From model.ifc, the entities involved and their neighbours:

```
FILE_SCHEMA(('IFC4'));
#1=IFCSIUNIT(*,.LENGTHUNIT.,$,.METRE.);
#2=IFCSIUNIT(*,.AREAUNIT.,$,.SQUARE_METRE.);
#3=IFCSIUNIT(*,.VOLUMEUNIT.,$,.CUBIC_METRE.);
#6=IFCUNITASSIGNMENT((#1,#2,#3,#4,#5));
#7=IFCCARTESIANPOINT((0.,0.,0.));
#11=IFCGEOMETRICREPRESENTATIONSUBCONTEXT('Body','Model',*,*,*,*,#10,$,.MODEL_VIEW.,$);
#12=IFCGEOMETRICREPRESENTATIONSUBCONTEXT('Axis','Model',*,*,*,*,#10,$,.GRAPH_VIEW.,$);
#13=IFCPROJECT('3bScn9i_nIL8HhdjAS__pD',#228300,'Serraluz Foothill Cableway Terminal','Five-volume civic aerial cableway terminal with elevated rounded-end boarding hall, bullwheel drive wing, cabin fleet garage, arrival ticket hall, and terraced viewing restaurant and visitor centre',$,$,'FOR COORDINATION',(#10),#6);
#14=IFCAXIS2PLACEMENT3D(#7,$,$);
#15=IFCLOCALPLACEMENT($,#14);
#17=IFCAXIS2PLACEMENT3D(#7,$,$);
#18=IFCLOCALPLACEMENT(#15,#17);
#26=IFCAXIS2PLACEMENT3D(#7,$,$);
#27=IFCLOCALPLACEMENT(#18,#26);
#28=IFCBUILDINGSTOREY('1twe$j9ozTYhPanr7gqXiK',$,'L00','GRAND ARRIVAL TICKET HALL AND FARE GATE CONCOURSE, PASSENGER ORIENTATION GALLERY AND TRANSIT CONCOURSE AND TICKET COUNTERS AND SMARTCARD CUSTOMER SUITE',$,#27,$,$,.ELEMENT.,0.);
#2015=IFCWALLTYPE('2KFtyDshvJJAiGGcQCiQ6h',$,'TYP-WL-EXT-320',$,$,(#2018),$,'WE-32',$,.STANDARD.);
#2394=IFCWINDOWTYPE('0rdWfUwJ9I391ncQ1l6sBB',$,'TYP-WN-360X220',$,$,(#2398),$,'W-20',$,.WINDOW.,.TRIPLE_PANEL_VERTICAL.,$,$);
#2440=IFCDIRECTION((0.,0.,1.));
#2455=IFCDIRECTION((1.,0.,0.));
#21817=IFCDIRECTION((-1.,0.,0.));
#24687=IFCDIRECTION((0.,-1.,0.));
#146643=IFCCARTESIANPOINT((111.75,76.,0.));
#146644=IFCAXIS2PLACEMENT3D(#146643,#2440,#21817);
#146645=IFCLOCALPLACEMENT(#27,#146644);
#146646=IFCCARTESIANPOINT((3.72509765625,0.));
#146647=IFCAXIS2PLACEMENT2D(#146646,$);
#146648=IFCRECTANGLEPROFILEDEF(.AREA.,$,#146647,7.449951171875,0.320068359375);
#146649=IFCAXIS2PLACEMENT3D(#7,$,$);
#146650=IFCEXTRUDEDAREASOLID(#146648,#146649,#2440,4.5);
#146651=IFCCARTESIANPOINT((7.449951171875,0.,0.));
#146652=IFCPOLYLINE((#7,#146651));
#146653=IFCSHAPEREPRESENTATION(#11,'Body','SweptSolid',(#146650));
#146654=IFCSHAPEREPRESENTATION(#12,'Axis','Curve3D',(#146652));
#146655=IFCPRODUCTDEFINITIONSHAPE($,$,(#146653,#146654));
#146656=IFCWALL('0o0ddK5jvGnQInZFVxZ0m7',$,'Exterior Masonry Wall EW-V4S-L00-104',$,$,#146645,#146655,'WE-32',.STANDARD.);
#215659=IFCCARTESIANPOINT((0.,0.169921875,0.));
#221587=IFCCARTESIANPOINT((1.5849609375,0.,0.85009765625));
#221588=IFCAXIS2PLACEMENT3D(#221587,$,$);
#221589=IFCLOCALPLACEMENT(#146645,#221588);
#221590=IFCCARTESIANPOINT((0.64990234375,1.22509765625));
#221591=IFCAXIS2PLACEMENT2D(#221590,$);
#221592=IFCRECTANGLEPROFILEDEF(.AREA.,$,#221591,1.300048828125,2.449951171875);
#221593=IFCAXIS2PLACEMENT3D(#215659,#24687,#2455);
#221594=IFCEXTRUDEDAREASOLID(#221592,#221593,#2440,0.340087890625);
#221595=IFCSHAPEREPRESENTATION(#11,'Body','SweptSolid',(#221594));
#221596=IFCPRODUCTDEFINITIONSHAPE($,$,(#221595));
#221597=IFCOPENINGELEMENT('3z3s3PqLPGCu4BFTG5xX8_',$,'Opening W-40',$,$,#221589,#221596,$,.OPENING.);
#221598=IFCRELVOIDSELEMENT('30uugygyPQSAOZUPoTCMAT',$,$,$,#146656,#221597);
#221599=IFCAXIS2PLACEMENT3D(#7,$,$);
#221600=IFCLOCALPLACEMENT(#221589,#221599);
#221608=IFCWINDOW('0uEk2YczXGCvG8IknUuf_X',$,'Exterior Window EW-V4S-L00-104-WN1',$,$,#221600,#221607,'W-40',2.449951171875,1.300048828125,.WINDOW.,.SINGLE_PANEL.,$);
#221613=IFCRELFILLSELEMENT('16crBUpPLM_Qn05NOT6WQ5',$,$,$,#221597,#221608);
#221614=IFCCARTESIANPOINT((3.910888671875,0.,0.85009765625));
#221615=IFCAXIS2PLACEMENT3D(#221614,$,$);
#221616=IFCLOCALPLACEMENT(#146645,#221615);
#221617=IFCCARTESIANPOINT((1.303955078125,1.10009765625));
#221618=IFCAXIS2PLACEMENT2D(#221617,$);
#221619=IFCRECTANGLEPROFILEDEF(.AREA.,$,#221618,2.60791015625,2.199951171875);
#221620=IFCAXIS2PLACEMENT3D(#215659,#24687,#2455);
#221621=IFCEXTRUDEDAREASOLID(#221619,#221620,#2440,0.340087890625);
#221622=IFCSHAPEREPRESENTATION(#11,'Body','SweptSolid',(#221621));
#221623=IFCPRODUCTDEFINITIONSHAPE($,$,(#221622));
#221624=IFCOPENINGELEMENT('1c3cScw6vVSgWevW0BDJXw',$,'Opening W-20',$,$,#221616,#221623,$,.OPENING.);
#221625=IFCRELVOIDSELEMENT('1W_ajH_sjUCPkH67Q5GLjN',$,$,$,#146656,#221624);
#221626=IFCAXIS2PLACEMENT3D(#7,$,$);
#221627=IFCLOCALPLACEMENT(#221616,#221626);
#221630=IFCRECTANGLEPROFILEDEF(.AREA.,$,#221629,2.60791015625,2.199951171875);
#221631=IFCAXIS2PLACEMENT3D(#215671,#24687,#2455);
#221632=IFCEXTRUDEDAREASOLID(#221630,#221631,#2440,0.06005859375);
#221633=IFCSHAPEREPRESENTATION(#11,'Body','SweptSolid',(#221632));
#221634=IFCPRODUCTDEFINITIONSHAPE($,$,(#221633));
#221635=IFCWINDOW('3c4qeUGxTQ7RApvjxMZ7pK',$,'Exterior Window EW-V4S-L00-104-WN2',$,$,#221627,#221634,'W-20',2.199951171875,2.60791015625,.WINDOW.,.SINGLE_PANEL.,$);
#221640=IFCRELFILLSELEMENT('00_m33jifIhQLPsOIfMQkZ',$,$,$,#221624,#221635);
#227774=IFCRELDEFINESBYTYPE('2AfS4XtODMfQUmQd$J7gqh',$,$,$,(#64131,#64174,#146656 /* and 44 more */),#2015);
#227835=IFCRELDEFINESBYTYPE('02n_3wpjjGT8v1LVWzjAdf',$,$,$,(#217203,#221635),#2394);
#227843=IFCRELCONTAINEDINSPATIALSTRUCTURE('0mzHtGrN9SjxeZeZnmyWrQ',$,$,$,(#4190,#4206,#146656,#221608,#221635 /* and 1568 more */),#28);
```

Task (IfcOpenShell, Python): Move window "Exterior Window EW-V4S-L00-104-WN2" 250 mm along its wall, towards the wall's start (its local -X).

```python
import ifcopenshell
import ifcopenshell.api.geometry
import ifcopenshell.util.placement
import ifcopenshell.util.unit

model = ifcopenshell.open("model.ifc")
unit_scale = ifcopenshell.util.unit.calculate_unit_scale(model)

window = model.by_guid("3c4qeUGxTQ7RApvjxMZ7pK")
opening = window.FillsVoids[0].RelatingOpeningElement
wall = opening.VoidsElements[0].RelatingBuildingElement

wall_matrix = ifcopenshell.util.placement.get_local_placement(wall.ObjectPlacement)
shift = wall_matrix[:3, 0] * -0.25 / unit_scale
before = ifcopenshell.util.placement.get_local_placement(window.ObjectPlacement)[:3, 3].copy()

# The window is placed relative to its opening, so it follows when the opening moves.
matrix = ifcopenshell.util.placement.get_local_placement(opening.ObjectPlacement)
matrix[:3, 3] += shift
ifcopenshell.api.geometry.edit_object_placement(
    model, product=opening, matrix=matrix, is_si=False, should_transform_children=True
)

after = ifcopenshell.util.placement.get_local_placement(window.ObjectPlacement)[:3, 3]
print("window moved by", (after - before).round(3) + 0.0)

model.write("model_edited.ifc")
```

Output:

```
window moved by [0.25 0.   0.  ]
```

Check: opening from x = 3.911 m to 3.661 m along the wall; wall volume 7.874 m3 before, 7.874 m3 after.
